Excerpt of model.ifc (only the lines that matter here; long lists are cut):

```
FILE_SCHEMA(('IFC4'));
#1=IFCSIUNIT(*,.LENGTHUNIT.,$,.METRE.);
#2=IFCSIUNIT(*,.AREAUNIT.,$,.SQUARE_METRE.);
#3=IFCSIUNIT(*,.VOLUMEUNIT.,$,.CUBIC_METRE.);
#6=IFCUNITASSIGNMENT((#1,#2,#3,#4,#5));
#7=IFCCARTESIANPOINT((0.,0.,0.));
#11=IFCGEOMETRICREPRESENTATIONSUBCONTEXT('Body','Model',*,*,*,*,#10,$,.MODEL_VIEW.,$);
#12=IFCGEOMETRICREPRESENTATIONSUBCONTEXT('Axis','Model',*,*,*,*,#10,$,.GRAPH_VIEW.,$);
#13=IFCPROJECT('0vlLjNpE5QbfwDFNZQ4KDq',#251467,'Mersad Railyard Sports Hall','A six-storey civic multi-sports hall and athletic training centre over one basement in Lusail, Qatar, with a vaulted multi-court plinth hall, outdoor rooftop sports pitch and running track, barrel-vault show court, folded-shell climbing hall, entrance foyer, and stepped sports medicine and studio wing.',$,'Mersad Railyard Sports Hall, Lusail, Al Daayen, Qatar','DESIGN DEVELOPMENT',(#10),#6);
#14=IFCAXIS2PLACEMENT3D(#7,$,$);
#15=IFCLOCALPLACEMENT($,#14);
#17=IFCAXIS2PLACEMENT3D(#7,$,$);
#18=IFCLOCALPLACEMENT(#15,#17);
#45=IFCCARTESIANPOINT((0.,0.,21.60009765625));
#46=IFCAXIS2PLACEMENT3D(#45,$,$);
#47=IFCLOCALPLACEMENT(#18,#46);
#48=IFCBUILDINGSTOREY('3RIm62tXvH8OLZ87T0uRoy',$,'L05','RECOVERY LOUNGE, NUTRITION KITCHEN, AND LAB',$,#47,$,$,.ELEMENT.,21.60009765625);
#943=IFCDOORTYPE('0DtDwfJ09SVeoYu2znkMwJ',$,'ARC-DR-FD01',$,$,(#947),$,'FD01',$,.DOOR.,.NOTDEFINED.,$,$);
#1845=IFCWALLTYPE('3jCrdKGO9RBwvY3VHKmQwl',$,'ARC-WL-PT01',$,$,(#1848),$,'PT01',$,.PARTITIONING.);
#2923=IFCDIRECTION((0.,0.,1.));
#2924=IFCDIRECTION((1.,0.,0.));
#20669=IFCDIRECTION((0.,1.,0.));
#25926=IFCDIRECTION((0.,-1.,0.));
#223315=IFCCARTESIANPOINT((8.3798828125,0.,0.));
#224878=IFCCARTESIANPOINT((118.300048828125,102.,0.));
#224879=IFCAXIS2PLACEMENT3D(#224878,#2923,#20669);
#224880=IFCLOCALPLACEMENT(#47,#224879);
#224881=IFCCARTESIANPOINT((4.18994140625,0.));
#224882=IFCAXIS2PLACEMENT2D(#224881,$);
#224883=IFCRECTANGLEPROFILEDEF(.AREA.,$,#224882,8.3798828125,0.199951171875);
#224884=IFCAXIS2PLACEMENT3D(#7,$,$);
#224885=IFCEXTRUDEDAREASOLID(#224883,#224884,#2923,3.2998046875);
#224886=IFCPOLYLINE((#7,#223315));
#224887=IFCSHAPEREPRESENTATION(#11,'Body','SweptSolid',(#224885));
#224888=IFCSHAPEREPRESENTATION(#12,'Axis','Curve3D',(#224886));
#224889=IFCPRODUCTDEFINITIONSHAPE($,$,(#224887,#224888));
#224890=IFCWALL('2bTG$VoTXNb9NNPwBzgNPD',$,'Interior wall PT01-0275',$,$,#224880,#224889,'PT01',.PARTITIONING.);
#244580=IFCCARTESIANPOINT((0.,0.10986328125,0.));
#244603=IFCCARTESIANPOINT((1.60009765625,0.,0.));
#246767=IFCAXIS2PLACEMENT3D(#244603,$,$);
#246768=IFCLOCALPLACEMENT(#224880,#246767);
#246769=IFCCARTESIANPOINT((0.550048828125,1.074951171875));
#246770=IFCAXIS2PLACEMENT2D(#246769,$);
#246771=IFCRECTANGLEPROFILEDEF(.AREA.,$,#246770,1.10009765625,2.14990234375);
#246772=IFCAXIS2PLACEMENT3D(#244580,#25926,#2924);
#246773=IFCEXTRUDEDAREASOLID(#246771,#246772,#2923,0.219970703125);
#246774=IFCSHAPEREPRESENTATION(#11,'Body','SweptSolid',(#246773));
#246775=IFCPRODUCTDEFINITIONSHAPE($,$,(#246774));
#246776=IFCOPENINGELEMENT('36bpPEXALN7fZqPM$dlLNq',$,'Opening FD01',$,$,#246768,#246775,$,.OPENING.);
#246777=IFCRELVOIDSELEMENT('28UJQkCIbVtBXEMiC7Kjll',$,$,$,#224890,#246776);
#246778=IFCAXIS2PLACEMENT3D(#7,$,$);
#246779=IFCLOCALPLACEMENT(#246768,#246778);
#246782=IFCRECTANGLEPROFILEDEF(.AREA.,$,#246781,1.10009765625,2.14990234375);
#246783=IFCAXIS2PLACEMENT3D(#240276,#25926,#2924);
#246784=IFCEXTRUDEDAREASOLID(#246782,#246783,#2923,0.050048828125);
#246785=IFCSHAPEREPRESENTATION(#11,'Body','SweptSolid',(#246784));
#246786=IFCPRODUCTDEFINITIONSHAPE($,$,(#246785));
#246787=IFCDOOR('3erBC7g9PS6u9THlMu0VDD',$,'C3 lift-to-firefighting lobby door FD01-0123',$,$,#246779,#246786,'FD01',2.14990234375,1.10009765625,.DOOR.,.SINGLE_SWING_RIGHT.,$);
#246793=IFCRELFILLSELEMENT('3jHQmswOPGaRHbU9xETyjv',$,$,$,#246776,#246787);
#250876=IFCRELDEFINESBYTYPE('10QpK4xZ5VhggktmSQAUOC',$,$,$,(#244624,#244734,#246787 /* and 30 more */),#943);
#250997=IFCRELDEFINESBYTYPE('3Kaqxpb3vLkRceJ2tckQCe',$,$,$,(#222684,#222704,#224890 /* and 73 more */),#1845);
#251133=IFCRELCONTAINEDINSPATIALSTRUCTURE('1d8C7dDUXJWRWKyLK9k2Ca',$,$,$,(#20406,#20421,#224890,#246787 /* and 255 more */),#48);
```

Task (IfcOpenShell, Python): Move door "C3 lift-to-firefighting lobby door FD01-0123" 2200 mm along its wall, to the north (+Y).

```python
import ifcopenshell
import ifcopenshell.api.geometry
import ifcopenshell.util.placement
import ifcopenshell.util.unit

model = ifcopenshell.open("model.ifc")
unit_scale = ifcopenshell.util.unit.calculate_unit_scale(model)

door = model.by_guid("3erBC7g9PS6u9THlMu0VDD")
opening = door.FillsVoids[0].RelatingOpeningElement
wall = opening.VoidsElements[0].RelatingBuildingElement

wall_matrix = ifcopenshell.util.placement.get_local_placement(wall.ObjectPlacement)
shift = wall_matrix[:3, 0] * 2.2 / unit_scale
before = ifcopenshell.util.placement.get_local_placement(door.ObjectPlacement)[:3, 3].copy()

# The door is placed relative to its opening, so it follows when the opening moves.
matrix = ifcopenshell.util.placement.get_local_placement(opening.ObjectPlacement)
matrix[:3, 3] += shift
ifcopenshell.api.geometry.edit_object_placement(
    model, product=opening, matrix=matrix, is_si=False, should_transform_children=True
)

after = ifcopenshell.util.placement.get_local_placement(door.ObjectPlacement)[:3, 3]
print("door moved by", (after - before).round(3) + 0.0)

model.write("model_v2.ifc")
```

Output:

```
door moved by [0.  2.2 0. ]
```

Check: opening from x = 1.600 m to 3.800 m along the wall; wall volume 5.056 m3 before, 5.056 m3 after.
